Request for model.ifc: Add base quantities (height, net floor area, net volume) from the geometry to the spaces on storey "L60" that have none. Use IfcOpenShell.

First a look at what the model holds.

```python
import ifcopenshell
import ifcopenshell.util.element
import ifcopenshell.util.unit

model = ifcopenshell.open("model.ifc")
print(model.schema)
for unit_type in ("LENGTHUNIT", "AREAUNIT", "VOLUMEUNIT"):
    print(unit_type, ifcopenshell.util.unit.calculate_unit_scale(model, unit_type))
storey = next(s for s in model.by_type("IfcBuildingStorey") if s.Name == "L60")
spaces = [e for e in ifcopenshell.util.element.get_decomposition(storey) if e.is_a("IfcSpace")]
for e in sorted(spaces, key=lambda e: e.id()):
    print(e.id(), e.is_a(), e.Name, list(ifcopenshell.util.element.get_psets(e, qtos_only=True)), sep=" | ")
```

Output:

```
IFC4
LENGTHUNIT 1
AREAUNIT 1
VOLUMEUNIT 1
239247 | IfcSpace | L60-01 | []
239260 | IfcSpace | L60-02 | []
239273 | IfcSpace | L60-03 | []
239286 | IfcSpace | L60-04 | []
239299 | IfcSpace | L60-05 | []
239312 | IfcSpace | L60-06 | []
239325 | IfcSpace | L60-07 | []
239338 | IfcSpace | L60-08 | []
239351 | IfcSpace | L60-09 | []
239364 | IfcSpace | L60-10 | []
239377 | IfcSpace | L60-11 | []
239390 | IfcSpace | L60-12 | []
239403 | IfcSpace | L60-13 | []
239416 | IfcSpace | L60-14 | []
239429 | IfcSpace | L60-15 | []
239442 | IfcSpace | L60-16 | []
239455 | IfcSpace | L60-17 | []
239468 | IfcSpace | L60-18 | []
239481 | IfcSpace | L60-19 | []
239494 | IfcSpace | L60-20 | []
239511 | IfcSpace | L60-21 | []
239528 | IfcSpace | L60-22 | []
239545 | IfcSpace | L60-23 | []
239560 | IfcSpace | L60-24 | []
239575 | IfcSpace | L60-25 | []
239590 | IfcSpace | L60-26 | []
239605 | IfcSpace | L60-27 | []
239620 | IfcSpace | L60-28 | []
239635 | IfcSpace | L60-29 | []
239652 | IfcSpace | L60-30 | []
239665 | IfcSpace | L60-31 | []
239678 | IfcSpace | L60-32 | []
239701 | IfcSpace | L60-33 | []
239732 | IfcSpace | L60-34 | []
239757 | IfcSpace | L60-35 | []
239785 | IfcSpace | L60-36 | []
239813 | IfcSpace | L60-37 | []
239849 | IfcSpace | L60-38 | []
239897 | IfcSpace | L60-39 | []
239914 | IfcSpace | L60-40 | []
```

```python
import ifcopenshell
import ifcopenshell.api.pset
import ifcopenshell.geom
import ifcopenshell.util.element
import ifcopenshell.util.shape
import ifcopenshell.util.unit

model = ifcopenshell.open("model.ifc")
unit_scale = ifcopenshell.util.unit.calculate_unit_scale(model)
area_scale = ifcopenshell.util.unit.calculate_unit_scale(model, "AREAUNIT")
volume_scale = ifcopenshell.util.unit.calculate_unit_scale(model, "VOLUMEUNIT")
settings = ifcopenshell.geom.settings()

storey = next(s for s in model.by_type("IfcBuildingStorey") if s.Name == "L60")
spaces = [e for e in ifcopenshell.util.element.get_decomposition(storey) if e.is_a("IfcSpace")]

for e in sorted(spaces, key=lambda e: e.id()):
    if ifcopenshell.util.element.get_psets(e, qtos_only=True, should_inherit=False):
        continue
    # Geometry comes back in metres, in the element's own axes.
    shape = ifcopenshell.geom.create_shape(settings, e)
    values = {
        "Height": ifcopenshell.util.shape.get_z(shape.geometry) / unit_scale,
        "NetFloorArea": ifcopenshell.util.shape.get_footprint_area(shape.geometry) / area_scale,
        "NetVolume": ifcopenshell.util.shape.get_volume(shape.geometry) / volume_scale,
    }
    qto = ifcopenshell.api.pset.add_qto(model, product=e, name="Qto_SpaceBaseQuantities")
    ifcopenshell.api.pset.edit_qto(model, qto=qto, properties=values)
    print(e.id(), {k: round(v, 3) for k, v in values.items()})

model.write("model_rev.ifc")
```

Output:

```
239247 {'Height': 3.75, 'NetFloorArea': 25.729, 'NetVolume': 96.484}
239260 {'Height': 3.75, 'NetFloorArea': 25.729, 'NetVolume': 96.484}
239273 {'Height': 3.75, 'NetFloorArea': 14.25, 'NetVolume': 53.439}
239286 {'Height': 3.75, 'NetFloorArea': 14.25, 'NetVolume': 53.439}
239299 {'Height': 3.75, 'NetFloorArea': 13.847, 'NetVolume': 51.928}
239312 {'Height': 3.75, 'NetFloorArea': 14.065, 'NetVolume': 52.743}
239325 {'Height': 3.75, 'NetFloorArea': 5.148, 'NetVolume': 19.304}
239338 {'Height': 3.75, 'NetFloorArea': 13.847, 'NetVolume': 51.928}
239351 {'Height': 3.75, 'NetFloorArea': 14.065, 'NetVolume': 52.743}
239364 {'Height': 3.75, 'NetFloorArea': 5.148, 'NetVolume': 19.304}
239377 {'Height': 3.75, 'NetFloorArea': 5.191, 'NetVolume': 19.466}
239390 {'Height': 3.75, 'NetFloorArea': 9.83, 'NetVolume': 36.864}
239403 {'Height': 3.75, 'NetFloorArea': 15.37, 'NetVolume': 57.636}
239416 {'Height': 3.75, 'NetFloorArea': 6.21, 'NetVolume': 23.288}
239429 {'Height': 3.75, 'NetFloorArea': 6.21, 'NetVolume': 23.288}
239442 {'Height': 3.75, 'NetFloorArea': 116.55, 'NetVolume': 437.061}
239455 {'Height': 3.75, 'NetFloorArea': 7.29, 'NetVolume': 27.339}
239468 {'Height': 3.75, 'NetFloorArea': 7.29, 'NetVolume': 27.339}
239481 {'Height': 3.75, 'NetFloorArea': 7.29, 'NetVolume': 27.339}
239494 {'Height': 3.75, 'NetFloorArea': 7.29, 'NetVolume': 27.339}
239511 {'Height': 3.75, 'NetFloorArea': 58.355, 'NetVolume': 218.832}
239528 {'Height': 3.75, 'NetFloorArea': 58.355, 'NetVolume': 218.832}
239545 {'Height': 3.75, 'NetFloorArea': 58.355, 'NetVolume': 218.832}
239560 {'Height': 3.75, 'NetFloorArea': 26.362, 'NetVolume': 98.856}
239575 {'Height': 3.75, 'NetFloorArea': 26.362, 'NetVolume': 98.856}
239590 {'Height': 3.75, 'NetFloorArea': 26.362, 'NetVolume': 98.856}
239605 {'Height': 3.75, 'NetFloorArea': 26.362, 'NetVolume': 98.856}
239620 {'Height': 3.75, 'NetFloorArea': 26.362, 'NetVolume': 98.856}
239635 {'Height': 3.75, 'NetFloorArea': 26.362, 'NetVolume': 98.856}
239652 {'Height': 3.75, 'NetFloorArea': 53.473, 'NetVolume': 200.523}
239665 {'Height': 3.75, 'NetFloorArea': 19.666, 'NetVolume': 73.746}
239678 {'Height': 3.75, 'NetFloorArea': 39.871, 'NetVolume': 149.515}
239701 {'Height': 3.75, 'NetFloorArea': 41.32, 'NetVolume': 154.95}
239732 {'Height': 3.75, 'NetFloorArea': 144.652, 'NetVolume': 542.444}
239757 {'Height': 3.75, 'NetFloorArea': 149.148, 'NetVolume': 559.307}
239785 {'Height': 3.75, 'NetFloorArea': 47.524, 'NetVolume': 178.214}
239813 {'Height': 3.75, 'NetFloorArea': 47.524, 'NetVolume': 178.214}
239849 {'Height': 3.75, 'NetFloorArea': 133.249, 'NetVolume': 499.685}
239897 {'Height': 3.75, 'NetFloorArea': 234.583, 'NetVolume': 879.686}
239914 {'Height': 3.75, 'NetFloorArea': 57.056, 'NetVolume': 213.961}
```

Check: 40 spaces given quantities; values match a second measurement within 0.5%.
